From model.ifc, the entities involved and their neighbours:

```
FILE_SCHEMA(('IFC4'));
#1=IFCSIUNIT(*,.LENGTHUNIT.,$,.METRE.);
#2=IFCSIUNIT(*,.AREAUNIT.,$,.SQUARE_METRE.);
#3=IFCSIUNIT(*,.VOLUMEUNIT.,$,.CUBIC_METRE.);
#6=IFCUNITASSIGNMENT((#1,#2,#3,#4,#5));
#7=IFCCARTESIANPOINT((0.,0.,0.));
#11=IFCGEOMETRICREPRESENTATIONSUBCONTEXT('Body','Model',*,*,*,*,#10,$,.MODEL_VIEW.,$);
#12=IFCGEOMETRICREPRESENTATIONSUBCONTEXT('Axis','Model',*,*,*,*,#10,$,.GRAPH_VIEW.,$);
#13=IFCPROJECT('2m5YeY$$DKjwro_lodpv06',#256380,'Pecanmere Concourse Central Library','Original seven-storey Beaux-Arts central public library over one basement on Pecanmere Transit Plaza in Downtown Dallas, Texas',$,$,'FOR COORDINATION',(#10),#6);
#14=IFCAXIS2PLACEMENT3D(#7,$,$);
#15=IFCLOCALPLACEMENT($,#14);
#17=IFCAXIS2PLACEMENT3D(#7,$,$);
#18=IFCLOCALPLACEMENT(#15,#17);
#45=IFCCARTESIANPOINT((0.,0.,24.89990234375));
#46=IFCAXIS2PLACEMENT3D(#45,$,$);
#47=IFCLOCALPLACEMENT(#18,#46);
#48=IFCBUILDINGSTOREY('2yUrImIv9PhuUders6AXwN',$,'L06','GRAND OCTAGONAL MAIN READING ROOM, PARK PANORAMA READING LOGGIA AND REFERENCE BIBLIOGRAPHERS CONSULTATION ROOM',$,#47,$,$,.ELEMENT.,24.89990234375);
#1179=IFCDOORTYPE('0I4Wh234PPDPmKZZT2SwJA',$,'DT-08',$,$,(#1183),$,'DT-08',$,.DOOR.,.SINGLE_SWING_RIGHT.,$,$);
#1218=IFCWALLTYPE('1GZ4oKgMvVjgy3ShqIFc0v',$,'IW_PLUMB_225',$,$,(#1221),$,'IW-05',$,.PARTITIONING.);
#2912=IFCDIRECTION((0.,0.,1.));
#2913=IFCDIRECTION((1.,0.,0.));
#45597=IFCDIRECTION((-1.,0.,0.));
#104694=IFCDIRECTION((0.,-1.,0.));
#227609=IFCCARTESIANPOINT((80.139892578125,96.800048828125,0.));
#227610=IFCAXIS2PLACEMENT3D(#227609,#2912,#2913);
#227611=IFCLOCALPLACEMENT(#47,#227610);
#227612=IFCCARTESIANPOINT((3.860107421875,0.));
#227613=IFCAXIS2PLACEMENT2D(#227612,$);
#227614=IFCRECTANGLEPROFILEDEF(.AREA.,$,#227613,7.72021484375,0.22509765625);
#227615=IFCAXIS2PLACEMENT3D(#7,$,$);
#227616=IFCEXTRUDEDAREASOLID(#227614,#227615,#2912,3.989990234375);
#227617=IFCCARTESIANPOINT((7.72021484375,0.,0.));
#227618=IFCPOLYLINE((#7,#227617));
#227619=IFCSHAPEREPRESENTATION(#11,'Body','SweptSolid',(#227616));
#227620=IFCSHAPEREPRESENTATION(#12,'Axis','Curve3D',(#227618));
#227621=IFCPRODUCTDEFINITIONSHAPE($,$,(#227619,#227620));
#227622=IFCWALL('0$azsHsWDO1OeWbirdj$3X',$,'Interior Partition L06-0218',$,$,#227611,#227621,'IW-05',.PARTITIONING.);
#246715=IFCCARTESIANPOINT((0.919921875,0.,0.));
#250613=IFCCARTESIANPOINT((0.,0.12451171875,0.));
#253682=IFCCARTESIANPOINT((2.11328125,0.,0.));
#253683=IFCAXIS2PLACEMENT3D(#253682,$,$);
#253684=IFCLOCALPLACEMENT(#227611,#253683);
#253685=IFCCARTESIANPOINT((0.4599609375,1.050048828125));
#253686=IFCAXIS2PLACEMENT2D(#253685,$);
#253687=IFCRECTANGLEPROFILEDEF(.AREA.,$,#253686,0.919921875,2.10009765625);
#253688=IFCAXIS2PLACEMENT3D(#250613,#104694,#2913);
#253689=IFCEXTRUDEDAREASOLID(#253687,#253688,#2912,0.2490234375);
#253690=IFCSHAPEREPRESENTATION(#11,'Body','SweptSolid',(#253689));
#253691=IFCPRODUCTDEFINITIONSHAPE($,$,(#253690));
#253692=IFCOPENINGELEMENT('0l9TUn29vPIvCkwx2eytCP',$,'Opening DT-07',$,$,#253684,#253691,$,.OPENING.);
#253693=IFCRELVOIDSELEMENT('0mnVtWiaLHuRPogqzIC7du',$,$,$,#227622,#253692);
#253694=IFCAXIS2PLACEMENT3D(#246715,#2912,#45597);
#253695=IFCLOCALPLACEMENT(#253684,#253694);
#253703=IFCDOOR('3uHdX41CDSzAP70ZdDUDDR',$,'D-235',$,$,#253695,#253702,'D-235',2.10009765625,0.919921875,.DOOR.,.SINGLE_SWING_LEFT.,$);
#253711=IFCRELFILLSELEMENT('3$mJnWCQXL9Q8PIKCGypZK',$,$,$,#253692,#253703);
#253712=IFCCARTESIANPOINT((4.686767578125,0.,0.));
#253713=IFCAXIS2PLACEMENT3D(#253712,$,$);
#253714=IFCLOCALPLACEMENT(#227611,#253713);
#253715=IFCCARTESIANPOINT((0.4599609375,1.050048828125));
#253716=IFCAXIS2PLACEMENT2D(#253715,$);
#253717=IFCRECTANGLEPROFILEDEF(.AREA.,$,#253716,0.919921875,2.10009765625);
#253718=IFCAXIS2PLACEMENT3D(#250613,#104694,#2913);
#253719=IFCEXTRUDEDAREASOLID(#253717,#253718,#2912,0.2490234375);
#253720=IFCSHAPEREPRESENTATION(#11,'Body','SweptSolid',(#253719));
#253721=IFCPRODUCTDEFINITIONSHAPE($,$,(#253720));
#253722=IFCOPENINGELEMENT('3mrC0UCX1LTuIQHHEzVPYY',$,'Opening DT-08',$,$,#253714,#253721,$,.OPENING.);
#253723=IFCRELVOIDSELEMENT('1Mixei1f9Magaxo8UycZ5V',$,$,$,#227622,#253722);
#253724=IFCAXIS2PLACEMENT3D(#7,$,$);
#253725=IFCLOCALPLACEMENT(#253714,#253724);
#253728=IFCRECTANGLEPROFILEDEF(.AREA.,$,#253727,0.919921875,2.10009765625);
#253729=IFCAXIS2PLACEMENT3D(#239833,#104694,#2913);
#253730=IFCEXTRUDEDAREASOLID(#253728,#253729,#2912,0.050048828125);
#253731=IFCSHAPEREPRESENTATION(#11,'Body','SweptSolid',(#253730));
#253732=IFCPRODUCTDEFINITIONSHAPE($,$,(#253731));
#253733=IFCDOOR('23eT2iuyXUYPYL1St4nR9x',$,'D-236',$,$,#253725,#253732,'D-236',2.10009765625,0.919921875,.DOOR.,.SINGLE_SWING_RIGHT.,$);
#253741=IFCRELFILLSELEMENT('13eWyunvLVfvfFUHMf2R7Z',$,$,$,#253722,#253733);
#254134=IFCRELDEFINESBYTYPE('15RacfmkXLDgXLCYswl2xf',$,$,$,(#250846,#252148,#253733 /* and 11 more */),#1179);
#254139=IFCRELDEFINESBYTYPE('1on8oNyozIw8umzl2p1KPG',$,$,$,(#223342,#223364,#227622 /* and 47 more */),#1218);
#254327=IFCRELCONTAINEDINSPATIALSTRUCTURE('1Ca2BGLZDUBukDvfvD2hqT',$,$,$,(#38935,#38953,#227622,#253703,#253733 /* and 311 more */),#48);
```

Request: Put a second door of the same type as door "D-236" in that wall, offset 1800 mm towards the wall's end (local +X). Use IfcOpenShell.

```python
import ifcopenshell
import ifcopenshell.api.feature
import ifcopenshell.api.geometry
import ifcopenshell.api.root
import ifcopenshell.geom
import ifcopenshell.util.element
import ifcopenshell.util.placement
import ifcopenshell.util.shape

model = ifcopenshell.open("model.ifc")
settings = ifcopenshell.geom.settings()


def volume(element):
    """Net volume in cubic metres, openings subtracted."""
    shape = ifcopenshell.geom.create_shape(settings, element)
    return ifcopenshell.util.shape.get_volume(shape.geometry)


door = model.by_guid("23eT2iuyXUYPYL1St4nR9x")
opening = door.FillsVoids[0].RelatingOpeningElement
wall = opening.VoidsElements[0].RelatingBuildingElement
before = volume(wall)
shift = ifcopenshell.util.placement.get_local_placement(wall.ObjectPlacement)[:3, 0] * 1.8

# copy_class copies the void relationship, type, container and properties, but no geometry.
new_opening = ifcopenshell.api.root.copy_class(model, product=opening)
new_opening.Representation = ifcopenshell.util.element.copy_deep(
    model, opening.Representation, exclude=["IfcGeometricRepresentationContext", "IfcRepresentationMap"]
)
new_door = ifcopenshell.api.root.copy_class(model, product=door)
new_door.Representation = ifcopenshell.util.element.copy_deep(
    model, door.Representation, exclude=["IfcGeometricRepresentationContext", "IfcRepresentationMap"]
)
new_door.Tag = None
ifcopenshell.api.feature.add_filling(model, opening=new_opening, element=new_door)

for old, new in ((opening, new_opening), (door, new_door)):
    matrix = ifcopenshell.util.placement.get_local_placement(old.ObjectPlacement)
    matrix[:3, 3] += shift
    ifcopenshell.api.geometry.edit_object_placement(model, product=new, matrix=matrix, is_si=False)

after = volume(wall)

print(f"wall volume {before:.3f} -> {after:.3f} m3")

model.write("model-out.ifc")
```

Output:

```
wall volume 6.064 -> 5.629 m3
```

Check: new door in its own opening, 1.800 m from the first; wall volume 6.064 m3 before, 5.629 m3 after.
